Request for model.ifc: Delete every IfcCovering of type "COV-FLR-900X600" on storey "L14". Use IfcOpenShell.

First a look at what the model holds.

```python
import ifcopenshell
import ifcopenshell.util.element

model = ifcopenshell.open("model.ifc")
print(model.schema)
storey = next(s for s in model.by_type("IfcBuildingStorey") if s.Name == "L14")
coverings = [e for e in ifcopenshell.util.element.get_decomposition(storey) if e.is_a("IfcCovering")]
seen = {}
for e in coverings:
    element_type = ifcopenshell.util.element.get_type(e)
    name = element_type.Name if element_type not in (None, e) else None
    seen[name] = seen.get(name, 0) + 1
for name, count in sorted(seen.items(), key=str):
    print(count, "x", name)
```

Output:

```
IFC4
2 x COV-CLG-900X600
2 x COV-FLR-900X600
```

```python
import ifcopenshell
import ifcopenshell.api.root
import ifcopenshell.util.element

model = ifcopenshell.open("model.ifc")

storey = next(s for s in model.by_type("IfcBuildingStorey") if s.Name == "L14")
coverings = [e for e in ifcopenshell.util.element.get_decomposition(storey) if e.is_a("IfcCovering")]
targets = [e for e in coverings if (t := ifcopenshell.util.element.get_type(e)) not in (None, e) and t.Name == "COV-FLR-900X600"]

for e in targets:
    ifcopenshell.api.root.remove_product(model, product=e)
print(len(targets), "removed")

model.write("model_v2.ifc")
```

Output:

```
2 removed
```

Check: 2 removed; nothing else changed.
